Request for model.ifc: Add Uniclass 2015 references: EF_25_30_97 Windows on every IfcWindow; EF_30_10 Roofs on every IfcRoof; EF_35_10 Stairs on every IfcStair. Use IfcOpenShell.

First a look at what the model holds.

```python
import ifcopenshell

model = ifcopenshell.open("model.ifc")
print(model.schema)
print("classifications:", [c.Name for c in model.by_type("IfcClassification")])
for ifc_class in ("IfcDoor", "IfcRoof", "IfcStair", "IfcWall", "IfcWindow"):
    print(ifc_class, len(model.by_type(ifc_class)))
```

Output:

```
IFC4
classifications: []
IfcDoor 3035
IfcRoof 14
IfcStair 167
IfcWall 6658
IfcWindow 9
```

```python
import ifcopenshell
import ifcopenshell.api.classification

model = ifcopenshell.open("model.ifc")

system = ifcopenshell.api.classification.add_classification(model, classification="Uniclass 2015")

codes = {
    "IfcWindow": ("EF_25_30_97", "Windows"),
    "IfcRoof": ("EF_30_10", "Roofs"),
    "IfcStair": ("EF_35_10", "Stairs"),
}
for ifc_class, (code, name) in codes.items():
    products = model.by_type(ifc_class)
    ifcopenshell.api.classification.add_reference(
        model, products=products, classification=system, identification=code, name=name
    )
    print(code, len(products))

model.write("model_updated.ifc")
```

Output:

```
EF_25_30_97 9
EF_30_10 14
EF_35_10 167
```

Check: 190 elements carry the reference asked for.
